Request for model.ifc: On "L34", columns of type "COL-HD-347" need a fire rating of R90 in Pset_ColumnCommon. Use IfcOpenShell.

First a look at what the model holds.

```python
import ifcopenshell
import ifcopenshell.util.element

model = ifcopenshell.open("model.ifc")
print(model.schema)
storey = next(s for s in model.by_type("IfcBuildingStorey") if s.Name == "L34")
columns = [e for e in ifcopenshell.util.element.get_decomposition(storey) if e.is_a("IfcColumn")]
seen = {}
for e in columns:
    element_type = ifcopenshell.util.element.get_type(e)
    key = (element_type.Name if element_type != e and element_type else None, ifcopenshell.util.element.get_pset(e, "Pset_ColumnCommon", "FireRating"))
    seen[key] = seen.get(key, 0) + 1
for (name, value), count in sorted(seen.items(), key=str):
    print(count, "x", name, "|", value)
```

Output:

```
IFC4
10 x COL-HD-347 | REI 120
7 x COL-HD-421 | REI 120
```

```python
import ifcopenshell
import ifcopenshell.api.pset
import ifcopenshell.util.element

model = ifcopenshell.open("model.ifc")

storey = next(s for s in model.by_type("IfcBuildingStorey") if s.Name == "L34")
columns = [e for e in ifcopenshell.util.element.get_decomposition(storey) if e.is_a("IfcColumn")]

count = 0
for e in columns:
    element_type = ifcopenshell.util.element.get_type(e)
    if element_type in (None, e) or element_type.Name != "COL-HD-347":
        continue
    found = ifcopenshell.util.element.get_pset(e, "Pset_ColumnCommon", should_inherit=False)
    if found:
        pset = model.by_id(found["id"])
        if len(ifcopenshell.util.element.get_elements_by_pset(pset)) > 1:
            pset = ifcopenshell.api.pset.unshare_pset(model, products=[e], pset=pset)[0]
    else:
        pset = ifcopenshell.api.pset.add_pset(model, product=e, name="Pset_ColumnCommon")
    ifcopenshell.api.pset.edit_pset(model, pset=pset, properties={"FireRating": "R90"})
    count += 1

print(count, "columns updated")

model.write("model_rev.ifc")
```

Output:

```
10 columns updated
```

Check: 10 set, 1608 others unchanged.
